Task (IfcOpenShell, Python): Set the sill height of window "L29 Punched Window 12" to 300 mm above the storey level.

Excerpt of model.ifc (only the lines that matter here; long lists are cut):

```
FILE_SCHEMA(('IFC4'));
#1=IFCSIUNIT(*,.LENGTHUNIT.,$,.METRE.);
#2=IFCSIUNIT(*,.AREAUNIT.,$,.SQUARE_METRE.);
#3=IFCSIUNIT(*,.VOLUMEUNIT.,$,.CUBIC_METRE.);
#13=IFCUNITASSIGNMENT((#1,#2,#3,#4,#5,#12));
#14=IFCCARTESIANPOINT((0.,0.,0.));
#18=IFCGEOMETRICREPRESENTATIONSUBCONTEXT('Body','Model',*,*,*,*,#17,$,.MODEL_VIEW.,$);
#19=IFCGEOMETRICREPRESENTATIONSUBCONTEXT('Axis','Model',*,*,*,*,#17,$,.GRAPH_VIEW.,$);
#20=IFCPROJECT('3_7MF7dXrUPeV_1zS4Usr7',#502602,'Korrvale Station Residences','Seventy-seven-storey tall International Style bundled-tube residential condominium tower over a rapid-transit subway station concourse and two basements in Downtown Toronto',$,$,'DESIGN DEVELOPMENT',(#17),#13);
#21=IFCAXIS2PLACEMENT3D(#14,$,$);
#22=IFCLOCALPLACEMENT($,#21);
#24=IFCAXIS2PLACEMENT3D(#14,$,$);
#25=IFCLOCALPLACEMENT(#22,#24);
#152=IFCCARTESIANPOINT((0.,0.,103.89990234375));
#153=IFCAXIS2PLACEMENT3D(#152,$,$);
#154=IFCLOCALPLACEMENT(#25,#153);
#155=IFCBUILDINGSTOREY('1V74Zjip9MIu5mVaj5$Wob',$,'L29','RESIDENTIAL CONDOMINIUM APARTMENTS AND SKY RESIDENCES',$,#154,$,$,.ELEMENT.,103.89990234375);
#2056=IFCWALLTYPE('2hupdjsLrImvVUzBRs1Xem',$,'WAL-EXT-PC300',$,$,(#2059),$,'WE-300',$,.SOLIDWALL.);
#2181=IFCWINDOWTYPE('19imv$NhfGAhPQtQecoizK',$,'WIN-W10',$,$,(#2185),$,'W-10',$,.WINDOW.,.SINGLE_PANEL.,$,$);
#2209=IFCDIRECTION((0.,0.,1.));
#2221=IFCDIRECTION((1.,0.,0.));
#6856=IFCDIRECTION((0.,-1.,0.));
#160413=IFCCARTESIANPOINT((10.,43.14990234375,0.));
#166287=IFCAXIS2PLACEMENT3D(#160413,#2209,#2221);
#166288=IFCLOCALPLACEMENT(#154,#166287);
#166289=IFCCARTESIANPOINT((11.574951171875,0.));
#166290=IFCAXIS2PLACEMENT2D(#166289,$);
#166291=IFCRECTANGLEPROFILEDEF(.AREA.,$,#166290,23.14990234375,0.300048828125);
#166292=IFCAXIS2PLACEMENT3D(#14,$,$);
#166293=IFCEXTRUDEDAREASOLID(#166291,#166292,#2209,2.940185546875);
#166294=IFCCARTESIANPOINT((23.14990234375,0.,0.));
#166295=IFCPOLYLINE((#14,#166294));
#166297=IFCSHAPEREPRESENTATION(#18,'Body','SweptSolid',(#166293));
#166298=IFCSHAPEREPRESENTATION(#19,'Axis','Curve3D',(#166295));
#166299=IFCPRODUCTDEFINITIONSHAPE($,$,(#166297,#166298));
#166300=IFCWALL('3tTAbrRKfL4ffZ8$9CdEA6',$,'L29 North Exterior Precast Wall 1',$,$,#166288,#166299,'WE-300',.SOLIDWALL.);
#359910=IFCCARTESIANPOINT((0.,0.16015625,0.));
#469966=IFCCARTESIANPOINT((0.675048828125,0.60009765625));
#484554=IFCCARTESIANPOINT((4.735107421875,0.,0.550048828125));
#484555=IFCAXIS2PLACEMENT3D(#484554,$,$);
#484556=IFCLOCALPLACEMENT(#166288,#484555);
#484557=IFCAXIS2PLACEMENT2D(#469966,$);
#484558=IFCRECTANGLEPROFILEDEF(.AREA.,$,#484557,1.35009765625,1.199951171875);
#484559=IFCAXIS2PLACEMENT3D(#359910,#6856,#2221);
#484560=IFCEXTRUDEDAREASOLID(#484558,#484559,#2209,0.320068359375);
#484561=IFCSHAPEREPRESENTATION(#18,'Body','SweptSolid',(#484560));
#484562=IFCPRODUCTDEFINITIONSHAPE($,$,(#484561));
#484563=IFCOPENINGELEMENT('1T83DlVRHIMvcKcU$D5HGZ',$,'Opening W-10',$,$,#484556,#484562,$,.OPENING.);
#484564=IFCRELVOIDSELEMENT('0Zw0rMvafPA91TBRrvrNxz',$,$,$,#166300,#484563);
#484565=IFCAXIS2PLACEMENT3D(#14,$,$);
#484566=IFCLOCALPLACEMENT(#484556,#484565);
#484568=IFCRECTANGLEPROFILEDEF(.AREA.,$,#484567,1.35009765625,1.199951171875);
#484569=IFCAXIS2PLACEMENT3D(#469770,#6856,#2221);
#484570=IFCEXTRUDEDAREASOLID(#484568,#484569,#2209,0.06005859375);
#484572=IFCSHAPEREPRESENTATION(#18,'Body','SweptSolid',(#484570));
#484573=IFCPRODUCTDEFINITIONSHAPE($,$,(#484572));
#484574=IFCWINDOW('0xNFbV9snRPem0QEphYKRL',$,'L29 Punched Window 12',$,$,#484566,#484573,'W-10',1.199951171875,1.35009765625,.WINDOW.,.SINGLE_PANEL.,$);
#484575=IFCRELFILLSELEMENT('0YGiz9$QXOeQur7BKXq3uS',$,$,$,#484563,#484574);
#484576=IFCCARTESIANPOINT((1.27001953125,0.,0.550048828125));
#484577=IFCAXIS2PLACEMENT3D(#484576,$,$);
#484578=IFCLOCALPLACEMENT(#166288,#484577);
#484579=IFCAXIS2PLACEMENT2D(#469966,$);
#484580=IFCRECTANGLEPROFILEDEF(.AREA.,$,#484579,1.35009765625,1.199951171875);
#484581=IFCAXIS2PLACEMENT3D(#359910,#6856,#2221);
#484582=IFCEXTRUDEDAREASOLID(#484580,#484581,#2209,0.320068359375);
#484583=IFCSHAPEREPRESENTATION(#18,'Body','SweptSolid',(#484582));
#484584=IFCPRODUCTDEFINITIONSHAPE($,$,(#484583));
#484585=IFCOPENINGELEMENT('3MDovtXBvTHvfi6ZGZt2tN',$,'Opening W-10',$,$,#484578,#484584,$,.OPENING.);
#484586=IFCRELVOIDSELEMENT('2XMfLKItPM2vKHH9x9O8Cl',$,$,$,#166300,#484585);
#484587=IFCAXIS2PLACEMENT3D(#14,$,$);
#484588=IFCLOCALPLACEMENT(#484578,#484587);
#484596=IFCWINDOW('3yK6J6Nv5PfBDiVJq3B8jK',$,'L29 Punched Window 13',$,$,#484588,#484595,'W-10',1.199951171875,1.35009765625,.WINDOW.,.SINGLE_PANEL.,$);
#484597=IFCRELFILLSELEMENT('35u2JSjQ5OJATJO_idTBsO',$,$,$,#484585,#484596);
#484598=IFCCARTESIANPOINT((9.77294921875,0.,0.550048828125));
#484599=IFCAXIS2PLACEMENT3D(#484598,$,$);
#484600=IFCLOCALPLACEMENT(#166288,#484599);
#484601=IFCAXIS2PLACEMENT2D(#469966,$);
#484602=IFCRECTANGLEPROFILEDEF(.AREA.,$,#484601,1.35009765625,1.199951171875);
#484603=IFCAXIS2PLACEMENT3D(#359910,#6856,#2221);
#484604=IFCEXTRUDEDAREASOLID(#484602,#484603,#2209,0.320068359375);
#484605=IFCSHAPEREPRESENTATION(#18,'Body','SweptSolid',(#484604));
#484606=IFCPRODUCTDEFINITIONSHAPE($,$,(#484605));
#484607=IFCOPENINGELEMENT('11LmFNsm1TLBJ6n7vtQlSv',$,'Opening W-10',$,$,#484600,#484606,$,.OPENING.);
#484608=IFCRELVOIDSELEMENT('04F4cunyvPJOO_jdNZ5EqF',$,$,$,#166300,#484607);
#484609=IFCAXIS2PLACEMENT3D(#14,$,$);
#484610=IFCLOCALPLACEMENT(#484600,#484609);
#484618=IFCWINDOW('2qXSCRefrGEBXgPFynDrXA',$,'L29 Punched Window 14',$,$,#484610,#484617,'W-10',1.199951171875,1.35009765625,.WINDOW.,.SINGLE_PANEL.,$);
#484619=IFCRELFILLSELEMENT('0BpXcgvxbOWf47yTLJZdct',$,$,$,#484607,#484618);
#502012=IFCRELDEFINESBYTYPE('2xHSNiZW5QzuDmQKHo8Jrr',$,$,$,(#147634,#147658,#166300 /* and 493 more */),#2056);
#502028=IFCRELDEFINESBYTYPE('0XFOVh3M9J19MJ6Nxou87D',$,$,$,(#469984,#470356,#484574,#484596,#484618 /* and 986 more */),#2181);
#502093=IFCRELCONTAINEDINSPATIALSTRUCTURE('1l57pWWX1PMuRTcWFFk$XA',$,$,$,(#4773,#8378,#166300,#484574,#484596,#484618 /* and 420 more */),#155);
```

```python
import numpy as np
import ifcopenshell
import ifcopenshell.api.geometry
import ifcopenshell.geom
import ifcopenshell.util.element
import ifcopenshell.util.placement
import ifcopenshell.util.shape
import ifcopenshell.util.unit

model = ifcopenshell.open("model.ifc")
unit_scale = ifcopenshell.util.unit.calculate_unit_scale(model)

window = model.by_guid("0xNFbV9snRPem0QEphYKRL")
opening = window.FillsVoids[0].RelatingOpeningElement
storey = ifcopenshell.util.element.get_container(window, ifc_class="IfcBuildingStorey")
level = ifcopenshell.util.placement.get_local_placement(storey.ObjectPlacement)[2, 3]

# The opening's origin need not be at the sill, so measure its lowest point.
shape = ifcopenshell.geom.create_shape(ifcopenshell.geom.settings(), opening)
bottom = ifcopenshell.util.shape.get_shape_bottom_elevation(shape, shape.geometry) / unit_scale
dz = level + 0.3 / unit_scale - bottom

shift = np.array([0.0, 0.0, dz])
# The window is placed relative to its opening, so it follows when the opening moves.
matrix = ifcopenshell.util.placement.get_local_placement(opening.ObjectPlacement)
matrix[:3, 3] += shift
ifcopenshell.api.geometry.edit_object_placement(
    model, product=opening, matrix=matrix, is_si=False, should_transform_children=True
)

print(f"moved by {dz * unit_scale:+.3f} m")

model.write("model_v2.ifc")
```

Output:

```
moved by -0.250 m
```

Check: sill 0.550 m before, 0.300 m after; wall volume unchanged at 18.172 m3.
